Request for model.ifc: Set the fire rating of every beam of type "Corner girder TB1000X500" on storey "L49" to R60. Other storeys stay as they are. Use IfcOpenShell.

First a look at what the model holds.

```python
import ifcopenshell
import ifcopenshell.util.element

model = ifcopenshell.open("model.ifc")
print(model.schema)
storey = next(s for s in model.by_type("IfcBuildingStorey") if s.Name == "L49")
beams = [e for e in ifcopenshell.util.element.get_decomposition(storey) if e.is_a("IfcBeam")]
seen = {}
for e in beams:
    element_type = ifcopenshell.util.element.get_type(e)
    key = (element_type.Name if element_type != e and element_type else None, ifcopenshell.util.element.get_pset(e, "Pset_BeamCommon", "FireRating"))
    seen[key] = seen.get(key, 0) + 1
for (name, value), count in sorted(seen.items(), key=str):
    print(count, "x", name, "|", value)
```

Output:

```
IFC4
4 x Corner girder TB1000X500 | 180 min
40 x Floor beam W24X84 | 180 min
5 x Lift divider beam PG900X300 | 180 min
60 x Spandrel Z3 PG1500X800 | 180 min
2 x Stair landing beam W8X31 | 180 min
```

```python
import ifcopenshell
import ifcopenshell.api.pset
import ifcopenshell.util.element

model = ifcopenshell.open("model.ifc")

storey = next(s for s in model.by_type("IfcBuildingStorey") if s.Name == "L49")
beams = [e for e in ifcopenshell.util.element.get_decomposition(storey) if e.is_a("IfcBeam")]

count = 0
for e in beams:
    element_type = ifcopenshell.util.element.get_type(e)
    if element_type in (None, e) or element_type.Name != "Corner girder TB1000X500":
        continue
    found = ifcopenshell.util.element.get_pset(e, "Pset_BeamCommon", should_inherit=False)
    if found:
        pset = model.by_id(found["id"])
        if len(ifcopenshell.util.element.get_elements_by_pset(pset)) > 1:
            pset = ifcopenshell.api.pset.unshare_pset(model, products=[e], pset=pset)[0]
    else:
        pset = ifcopenshell.api.pset.add_pset(model, product=e, name="Pset_BeamCommon")
    ifcopenshell.api.pset.edit_pset(model, pset=pset, properties={"FireRating": "R60"})
    count += 1

print(count, "beams updated")

model.write("model_updated.ifc")
```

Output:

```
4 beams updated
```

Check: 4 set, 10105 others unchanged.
